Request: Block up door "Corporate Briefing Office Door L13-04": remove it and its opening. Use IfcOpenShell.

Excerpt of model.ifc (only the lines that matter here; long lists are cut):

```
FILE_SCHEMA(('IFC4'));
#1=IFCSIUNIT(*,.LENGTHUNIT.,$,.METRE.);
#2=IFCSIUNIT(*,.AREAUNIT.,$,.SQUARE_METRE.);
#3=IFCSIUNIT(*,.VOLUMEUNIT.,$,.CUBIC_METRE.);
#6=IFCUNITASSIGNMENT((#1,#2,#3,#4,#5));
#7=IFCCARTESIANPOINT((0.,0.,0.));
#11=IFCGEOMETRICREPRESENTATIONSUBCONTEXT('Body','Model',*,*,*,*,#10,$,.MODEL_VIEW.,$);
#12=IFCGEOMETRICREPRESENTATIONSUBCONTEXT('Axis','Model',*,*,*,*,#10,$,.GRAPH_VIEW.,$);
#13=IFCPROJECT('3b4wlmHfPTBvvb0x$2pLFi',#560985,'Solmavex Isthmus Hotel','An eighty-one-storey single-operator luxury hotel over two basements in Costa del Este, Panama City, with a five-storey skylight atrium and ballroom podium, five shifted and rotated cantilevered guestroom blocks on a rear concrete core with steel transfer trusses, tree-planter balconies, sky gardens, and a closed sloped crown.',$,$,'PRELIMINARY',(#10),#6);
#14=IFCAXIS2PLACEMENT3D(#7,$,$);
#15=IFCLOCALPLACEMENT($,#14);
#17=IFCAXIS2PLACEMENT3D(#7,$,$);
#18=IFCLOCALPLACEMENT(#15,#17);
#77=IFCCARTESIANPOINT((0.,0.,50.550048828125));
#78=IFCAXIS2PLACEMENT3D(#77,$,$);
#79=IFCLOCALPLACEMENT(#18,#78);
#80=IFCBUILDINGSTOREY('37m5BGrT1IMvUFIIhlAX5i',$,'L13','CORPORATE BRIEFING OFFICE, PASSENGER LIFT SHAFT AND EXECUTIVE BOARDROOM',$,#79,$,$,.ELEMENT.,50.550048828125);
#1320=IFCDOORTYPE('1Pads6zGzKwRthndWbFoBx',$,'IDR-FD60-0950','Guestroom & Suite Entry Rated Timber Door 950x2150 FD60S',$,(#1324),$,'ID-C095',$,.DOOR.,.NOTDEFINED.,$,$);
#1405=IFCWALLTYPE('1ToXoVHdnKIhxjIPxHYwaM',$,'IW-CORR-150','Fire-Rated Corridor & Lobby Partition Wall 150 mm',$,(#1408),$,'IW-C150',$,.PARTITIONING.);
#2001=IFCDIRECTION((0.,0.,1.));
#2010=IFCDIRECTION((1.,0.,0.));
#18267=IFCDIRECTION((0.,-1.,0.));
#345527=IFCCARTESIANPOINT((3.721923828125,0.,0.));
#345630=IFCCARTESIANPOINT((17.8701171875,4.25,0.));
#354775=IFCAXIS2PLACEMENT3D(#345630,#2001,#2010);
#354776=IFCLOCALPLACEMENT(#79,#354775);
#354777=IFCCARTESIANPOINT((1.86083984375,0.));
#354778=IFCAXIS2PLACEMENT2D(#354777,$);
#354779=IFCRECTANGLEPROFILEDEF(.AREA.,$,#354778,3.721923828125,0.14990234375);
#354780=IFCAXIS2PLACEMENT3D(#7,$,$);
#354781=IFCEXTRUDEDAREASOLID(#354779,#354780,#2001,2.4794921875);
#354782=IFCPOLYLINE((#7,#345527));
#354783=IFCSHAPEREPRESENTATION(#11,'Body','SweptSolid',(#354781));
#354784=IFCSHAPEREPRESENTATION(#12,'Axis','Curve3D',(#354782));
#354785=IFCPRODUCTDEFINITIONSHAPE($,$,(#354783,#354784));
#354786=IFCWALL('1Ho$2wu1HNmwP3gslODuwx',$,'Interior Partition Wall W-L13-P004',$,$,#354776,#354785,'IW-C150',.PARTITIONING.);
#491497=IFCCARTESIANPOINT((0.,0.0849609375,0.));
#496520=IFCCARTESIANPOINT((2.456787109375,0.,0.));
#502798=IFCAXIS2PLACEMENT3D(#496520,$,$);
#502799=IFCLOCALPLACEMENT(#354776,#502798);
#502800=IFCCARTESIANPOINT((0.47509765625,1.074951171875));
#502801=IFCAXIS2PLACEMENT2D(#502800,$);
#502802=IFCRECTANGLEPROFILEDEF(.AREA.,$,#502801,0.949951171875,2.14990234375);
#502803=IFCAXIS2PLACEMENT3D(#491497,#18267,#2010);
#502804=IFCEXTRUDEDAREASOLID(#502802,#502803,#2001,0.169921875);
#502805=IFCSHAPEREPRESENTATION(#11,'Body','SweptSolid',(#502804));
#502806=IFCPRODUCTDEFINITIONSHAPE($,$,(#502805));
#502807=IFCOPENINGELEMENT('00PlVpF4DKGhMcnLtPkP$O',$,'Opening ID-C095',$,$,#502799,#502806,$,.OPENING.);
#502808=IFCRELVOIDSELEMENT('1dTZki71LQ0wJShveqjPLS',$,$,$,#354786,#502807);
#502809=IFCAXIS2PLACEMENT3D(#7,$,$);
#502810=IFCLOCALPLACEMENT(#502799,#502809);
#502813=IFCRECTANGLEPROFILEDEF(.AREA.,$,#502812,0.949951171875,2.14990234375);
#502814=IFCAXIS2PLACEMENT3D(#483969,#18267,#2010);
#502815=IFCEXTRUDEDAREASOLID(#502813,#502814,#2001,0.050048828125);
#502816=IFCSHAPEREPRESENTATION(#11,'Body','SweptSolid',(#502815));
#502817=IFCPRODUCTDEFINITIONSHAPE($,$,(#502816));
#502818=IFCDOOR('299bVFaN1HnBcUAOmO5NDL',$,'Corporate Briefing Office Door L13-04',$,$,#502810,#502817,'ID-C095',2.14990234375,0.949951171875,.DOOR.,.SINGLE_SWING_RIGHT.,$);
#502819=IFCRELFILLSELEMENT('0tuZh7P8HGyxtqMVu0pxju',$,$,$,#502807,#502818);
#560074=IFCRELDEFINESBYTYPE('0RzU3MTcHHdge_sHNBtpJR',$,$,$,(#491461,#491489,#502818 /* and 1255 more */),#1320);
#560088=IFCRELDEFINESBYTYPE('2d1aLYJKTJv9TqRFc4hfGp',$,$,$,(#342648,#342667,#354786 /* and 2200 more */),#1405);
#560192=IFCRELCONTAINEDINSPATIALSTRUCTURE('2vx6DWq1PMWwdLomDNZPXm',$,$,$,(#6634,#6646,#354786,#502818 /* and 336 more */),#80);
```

```python
import ifcopenshell
import ifcopenshell.api.feature
import ifcopenshell.api.root
import ifcopenshell.geom
import ifcopenshell.util.shape

model = ifcopenshell.open("model.ifc")
settings = ifcopenshell.geom.settings()


def volume(element):
    """Net volume in cubic metres, openings subtracted."""
    shape = ifcopenshell.geom.create_shape(settings, element)
    return ifcopenshell.util.shape.get_volume(shape.geometry)


door = model.by_guid("299bVFaN1HnBcUAOmO5NDL")
opening = door.FillsVoids[0].RelatingOpeningElement
wall = opening.VoidsElements[0].RelatingBuildingElement
before = volume(wall)

ifcopenshell.api.root.remove_product(model, product=door)
ifcopenshell.api.feature.remove_feature(model, feature=opening)

after = volume(wall)

print(f"wall volume {before:.3f} -> {after:.3f} m3")

model.write("model_edited.ifc")
```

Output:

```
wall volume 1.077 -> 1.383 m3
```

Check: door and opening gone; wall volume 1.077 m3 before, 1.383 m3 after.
